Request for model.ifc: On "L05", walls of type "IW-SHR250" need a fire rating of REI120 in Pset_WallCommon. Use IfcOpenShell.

First a look at what the model holds.

```python
import ifcopenshell
import ifcopenshell.util.element

model = ifcopenshell.open("model.ifc")
print(model.schema)
storey = next(s for s in model.by_type("IfcBuildingStorey") if s.Name == "L05")
walls = [e for e in ifcopenshell.util.element.get_decomposition(storey) if e.is_a("IfcWall")]
seen = {}
for e in walls:
    element_type = ifcopenshell.util.element.get_type(e)
    key = (element_type.Name if element_type != e and element_type else None, ifcopenshell.util.element.get_pset(e, "Pset_WallCommon", "FireRating"))
    seen[key] = seen.get(key, 0) + 1
for (name, value), count in sorted(seen.items(), key=str):
    print(count, "x", name, "|", value)
```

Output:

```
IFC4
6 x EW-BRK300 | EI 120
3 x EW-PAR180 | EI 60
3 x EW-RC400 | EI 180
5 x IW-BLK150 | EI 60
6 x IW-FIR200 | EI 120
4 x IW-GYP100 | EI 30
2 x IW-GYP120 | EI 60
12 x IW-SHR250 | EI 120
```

```python
import ifcopenshell
import ifcopenshell.api.pset
import ifcopenshell.util.element

model = ifcopenshell.open("model.ifc")

storey = next(s for s in model.by_type("IfcBuildingStorey") if s.Name == "L05")
walls = [e for e in ifcopenshell.util.element.get_decomposition(storey) if e.is_a("IfcWall")]

count = 0
for e in walls:
    element_type = ifcopenshell.util.element.get_type(e)
    if element_type in (None, e) or element_type.Name != "IW-SHR250":
        continue
    # add_pset returns the element's existing set when there is one.
    pset = ifcopenshell.api.pset.add_pset(model, product=e, name="Pset_WallCommon")
    ifcopenshell.api.pset.edit_pset(model, pset=pset, properties={"FireRating": "REI120"})
    count += 1

print(count, "walls updated")

model.write("model-out.ifc")
```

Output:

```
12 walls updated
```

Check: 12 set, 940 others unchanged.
